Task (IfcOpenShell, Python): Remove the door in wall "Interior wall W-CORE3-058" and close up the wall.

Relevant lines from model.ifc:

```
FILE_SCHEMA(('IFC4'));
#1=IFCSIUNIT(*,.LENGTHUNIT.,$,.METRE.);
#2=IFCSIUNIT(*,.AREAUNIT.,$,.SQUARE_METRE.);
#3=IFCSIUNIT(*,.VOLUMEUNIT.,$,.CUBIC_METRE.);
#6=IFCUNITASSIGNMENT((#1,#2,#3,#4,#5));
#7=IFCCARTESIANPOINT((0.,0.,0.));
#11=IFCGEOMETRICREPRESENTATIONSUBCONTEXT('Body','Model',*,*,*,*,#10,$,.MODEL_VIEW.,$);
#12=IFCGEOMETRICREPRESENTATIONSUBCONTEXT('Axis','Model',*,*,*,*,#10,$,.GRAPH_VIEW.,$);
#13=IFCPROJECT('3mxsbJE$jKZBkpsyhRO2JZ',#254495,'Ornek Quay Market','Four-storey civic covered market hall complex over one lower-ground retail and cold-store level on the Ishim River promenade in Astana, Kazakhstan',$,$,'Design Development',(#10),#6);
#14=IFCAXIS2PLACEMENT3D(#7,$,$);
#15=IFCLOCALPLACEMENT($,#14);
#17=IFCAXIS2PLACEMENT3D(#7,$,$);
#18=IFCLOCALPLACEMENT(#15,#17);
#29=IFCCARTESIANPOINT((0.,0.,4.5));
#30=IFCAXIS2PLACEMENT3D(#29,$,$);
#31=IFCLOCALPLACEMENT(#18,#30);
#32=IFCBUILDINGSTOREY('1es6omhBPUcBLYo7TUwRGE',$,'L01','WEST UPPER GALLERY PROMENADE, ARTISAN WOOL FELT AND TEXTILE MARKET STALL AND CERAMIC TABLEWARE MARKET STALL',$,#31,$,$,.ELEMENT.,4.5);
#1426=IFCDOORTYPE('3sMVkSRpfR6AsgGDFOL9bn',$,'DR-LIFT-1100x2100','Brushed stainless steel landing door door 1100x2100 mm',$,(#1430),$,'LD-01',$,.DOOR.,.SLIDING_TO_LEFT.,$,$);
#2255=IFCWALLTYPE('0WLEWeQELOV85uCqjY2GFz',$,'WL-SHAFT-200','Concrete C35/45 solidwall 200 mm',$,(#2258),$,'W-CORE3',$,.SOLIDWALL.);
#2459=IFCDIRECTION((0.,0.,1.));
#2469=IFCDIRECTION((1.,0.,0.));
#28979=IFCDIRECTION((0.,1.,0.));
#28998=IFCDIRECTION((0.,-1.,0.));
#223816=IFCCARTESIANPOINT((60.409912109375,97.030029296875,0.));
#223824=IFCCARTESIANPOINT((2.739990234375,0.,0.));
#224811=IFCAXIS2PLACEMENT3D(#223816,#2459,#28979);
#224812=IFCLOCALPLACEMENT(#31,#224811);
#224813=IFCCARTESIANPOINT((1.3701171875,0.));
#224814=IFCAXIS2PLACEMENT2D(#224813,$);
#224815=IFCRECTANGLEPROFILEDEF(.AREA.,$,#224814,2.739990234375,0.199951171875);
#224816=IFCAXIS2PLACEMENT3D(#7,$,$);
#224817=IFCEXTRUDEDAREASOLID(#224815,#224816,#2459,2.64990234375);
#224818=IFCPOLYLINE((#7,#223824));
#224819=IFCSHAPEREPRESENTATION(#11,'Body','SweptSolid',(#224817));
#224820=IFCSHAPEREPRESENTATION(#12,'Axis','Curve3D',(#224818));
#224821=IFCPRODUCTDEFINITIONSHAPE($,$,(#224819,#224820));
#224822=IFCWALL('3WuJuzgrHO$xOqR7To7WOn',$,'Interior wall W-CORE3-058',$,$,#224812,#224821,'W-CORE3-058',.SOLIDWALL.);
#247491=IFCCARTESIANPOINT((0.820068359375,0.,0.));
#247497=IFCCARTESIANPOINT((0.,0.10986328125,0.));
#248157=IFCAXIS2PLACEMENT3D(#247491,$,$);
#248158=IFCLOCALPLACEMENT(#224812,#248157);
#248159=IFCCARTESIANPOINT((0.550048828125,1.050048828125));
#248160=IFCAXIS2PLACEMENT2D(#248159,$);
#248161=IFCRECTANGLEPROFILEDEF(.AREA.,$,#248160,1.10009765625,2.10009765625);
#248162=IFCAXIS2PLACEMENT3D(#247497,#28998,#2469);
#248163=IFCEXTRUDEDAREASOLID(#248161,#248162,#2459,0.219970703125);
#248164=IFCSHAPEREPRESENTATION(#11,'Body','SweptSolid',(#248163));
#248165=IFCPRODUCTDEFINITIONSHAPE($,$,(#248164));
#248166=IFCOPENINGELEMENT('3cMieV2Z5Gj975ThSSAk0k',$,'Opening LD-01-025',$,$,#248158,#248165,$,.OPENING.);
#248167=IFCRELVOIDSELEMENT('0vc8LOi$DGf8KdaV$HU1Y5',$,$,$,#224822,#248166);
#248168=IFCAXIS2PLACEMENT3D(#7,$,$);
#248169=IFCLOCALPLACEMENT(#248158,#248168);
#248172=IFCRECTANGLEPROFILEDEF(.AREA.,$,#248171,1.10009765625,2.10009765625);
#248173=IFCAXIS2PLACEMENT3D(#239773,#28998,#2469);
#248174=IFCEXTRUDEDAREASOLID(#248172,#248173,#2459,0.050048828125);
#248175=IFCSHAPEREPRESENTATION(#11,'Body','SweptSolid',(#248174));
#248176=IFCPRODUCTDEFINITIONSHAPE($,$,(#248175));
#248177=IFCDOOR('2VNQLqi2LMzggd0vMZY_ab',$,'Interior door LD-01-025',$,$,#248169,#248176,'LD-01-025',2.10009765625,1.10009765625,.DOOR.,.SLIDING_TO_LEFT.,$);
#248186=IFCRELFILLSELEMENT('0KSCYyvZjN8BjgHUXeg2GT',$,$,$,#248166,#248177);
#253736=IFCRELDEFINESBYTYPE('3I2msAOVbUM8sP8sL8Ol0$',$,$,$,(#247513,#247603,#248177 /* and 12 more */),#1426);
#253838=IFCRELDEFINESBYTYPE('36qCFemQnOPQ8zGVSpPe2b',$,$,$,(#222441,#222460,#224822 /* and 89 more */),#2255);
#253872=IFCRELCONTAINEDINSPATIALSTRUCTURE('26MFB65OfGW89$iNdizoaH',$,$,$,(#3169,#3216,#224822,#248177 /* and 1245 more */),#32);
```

```python
import ifcopenshell
import ifcopenshell.api.feature
import ifcopenshell.api.root
import ifcopenshell.geom
import ifcopenshell.util.shape

model = ifcopenshell.open("model.ifc")
settings = ifcopenshell.geom.settings()


def volume(element):
    """Net volume in cubic metres, openings subtracted."""
    shape = ifcopenshell.geom.create_shape(settings, element)
    return ifcopenshell.util.shape.get_volume(shape.geometry)


door = model.by_guid("2VNQLqi2LMzggd0vMZY_ab")
opening = door.FillsVoids[0].RelatingOpeningElement
wall = opening.VoidsElements[0].RelatingBuildingElement
before = volume(wall)

ifcopenshell.api.root.remove_product(model, product=door)
ifcopenshell.api.feature.remove_feature(model, feature=opening)

after = volume(wall)

print(f"wall volume {before:.3f} -> {after:.3f} m3")

model.write("model-out.ifc")
```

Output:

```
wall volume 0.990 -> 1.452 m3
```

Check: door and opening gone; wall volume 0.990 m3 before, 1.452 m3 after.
